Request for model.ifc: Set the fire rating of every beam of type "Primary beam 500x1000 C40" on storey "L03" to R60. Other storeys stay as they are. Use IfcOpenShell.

First a look at what the model holds.

```python
import ifcopenshell
import ifcopenshell.util.element

model = ifcopenshell.open("model.ifc")
print(model.schema)
storey = next(s for s in model.by_type("IfcBuildingStorey") if s.Name == "L03")
beams = [e for e in ifcopenshell.util.element.get_decomposition(storey) if e.is_a("IfcBeam")]
seen = {}
for e in beams:
    element_type = ifcopenshell.util.element.get_type(e)
    key = (element_type.Name if element_type != e and element_type else None, ifcopenshell.util.element.get_pset(e, "Pset_BeamCommon", "FireRating"))
    seen[key] = seen.get(key, 0) + 1
for (name, value), count in sorted(seen.items(), key=str):
    print(count, "x", name, "|", value)
```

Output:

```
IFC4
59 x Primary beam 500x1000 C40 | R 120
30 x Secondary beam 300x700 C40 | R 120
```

```python
import ifcopenshell
import ifcopenshell.api.pset
import ifcopenshell.util.element

model = ifcopenshell.open("model.ifc")

storey = next(s for s in model.by_type("IfcBuildingStorey") if s.Name == "L03")
beams = [e for e in ifcopenshell.util.element.get_decomposition(storey) if e.is_a("IfcBeam")]

count = 0
for e in beams:
    element_type = ifcopenshell.util.element.get_type(e)
    if element_type in (None, e) or element_type.Name != "Primary beam 500x1000 C40":
        continue
    # add_pset returns the element's existing set when there is one.
    pset = ifcopenshell.api.pset.add_pset(model, product=e, name="Pset_BeamCommon")
    ifcopenshell.api.pset.edit_pset(model, pset=pset, properties={"FireRating": "R60"})
    count += 1

print(count, "beams updated")

model.write("model_edited.ifc")
```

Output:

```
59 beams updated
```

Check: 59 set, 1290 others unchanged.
